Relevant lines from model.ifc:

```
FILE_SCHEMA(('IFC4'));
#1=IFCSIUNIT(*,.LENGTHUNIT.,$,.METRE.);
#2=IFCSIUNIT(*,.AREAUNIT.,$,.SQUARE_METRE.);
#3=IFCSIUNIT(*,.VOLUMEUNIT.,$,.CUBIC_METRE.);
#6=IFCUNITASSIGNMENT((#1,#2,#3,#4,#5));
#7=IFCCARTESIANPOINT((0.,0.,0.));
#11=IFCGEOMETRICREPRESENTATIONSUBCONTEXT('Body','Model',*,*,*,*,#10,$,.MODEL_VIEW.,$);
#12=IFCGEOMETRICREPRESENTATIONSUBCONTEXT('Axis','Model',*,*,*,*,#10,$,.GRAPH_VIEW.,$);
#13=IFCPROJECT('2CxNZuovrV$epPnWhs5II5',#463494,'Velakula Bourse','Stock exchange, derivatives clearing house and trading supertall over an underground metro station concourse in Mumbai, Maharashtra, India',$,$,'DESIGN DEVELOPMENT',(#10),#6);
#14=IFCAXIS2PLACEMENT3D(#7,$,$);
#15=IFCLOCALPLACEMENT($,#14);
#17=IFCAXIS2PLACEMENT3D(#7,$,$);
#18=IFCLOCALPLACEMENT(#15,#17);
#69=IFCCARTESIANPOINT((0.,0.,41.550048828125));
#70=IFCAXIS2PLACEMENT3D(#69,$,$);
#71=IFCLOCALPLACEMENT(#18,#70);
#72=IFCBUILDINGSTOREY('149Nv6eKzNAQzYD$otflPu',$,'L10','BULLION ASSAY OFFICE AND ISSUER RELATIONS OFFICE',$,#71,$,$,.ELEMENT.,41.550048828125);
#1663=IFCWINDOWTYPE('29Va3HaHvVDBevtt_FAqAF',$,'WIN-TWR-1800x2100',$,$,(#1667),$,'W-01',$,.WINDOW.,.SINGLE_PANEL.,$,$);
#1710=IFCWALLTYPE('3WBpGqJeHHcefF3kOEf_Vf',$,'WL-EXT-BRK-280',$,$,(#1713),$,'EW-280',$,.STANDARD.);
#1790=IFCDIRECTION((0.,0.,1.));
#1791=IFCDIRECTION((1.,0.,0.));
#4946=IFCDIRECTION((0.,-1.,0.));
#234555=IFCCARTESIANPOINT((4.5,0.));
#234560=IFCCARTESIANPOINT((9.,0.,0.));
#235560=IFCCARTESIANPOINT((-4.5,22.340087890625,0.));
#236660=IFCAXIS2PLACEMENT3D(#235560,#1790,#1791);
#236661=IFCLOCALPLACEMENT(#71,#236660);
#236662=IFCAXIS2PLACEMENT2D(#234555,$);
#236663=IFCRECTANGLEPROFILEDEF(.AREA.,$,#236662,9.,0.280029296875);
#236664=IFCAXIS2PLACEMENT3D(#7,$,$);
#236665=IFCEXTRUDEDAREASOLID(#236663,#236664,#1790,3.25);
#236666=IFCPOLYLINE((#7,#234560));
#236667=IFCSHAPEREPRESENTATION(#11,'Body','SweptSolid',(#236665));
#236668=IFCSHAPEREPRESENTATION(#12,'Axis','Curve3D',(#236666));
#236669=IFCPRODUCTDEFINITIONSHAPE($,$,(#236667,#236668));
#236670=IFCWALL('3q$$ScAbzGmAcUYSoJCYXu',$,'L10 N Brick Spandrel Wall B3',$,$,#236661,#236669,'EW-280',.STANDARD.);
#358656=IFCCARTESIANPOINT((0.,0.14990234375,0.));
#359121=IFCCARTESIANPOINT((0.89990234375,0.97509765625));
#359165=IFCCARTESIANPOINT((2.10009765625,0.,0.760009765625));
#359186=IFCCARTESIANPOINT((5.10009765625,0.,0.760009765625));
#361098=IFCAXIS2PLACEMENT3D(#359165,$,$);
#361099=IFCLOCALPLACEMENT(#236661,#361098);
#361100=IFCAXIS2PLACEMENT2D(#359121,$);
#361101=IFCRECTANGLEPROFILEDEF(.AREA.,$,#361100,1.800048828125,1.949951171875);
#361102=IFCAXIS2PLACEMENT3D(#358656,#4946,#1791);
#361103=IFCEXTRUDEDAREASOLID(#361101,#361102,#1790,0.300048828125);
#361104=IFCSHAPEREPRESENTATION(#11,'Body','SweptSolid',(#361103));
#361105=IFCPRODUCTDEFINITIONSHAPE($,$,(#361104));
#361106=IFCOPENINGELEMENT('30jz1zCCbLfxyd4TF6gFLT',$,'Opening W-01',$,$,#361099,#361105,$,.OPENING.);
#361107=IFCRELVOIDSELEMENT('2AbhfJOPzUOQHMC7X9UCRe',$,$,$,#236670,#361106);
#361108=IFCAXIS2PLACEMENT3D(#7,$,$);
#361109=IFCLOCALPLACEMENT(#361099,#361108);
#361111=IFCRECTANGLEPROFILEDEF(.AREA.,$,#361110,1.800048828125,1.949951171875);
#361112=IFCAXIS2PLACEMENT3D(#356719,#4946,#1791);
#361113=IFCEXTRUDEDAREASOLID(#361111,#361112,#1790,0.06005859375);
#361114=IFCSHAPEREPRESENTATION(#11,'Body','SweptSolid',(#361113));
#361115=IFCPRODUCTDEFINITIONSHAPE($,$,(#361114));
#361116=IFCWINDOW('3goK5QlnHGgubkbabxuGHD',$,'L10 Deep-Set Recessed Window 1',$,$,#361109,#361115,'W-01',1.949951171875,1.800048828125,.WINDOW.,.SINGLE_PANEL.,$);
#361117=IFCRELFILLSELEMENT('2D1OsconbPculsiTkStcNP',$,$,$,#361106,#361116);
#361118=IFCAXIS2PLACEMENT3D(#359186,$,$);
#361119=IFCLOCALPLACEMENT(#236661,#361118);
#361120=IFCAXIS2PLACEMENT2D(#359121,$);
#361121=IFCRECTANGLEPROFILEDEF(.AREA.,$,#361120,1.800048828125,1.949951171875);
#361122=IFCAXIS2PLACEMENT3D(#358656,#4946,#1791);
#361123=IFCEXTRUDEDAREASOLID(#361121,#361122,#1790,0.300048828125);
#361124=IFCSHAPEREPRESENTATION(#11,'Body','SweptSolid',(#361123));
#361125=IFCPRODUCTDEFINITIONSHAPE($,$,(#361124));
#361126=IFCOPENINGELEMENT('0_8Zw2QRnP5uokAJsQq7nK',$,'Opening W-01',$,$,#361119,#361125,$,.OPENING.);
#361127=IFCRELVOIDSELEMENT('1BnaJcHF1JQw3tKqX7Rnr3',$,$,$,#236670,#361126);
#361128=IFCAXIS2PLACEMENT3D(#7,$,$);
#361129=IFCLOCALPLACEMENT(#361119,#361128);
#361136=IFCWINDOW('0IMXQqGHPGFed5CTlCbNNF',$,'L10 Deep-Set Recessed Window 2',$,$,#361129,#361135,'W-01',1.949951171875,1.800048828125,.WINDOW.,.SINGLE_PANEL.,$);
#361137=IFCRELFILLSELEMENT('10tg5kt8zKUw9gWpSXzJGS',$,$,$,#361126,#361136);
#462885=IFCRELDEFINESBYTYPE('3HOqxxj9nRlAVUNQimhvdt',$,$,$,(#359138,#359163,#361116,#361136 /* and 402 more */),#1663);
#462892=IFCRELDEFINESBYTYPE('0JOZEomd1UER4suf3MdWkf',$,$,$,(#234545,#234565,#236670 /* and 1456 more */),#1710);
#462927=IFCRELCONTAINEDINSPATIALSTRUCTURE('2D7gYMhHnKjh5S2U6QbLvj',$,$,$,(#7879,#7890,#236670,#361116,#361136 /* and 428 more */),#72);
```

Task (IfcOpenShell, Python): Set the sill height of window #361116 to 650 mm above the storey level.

```python
import numpy as np
import ifcopenshell
import ifcopenshell.api.geometry
import ifcopenshell.geom
import ifcopenshell.util.element
import ifcopenshell.util.placement
import ifcopenshell.util.shape
import ifcopenshell.util.unit

model = ifcopenshell.open("model.ifc")
unit_scale = ifcopenshell.util.unit.calculate_unit_scale(model)

window = model.by_guid("3goK5QlnHGgubkbabxuGHD")
opening = window.FillsVoids[0].RelatingOpeningElement
storey = ifcopenshell.util.element.get_container(window, ifc_class="IfcBuildingStorey")
level = ifcopenshell.util.placement.get_local_placement(storey.ObjectPlacement)[2, 3]

# The opening's origin need not be at the sill, so measure its lowest point.
shape = ifcopenshell.geom.create_shape(ifcopenshell.geom.settings(), opening)
bottom = ifcopenshell.util.shape.get_shape_bottom_elevation(shape, shape.geometry) / unit_scale
dz = level + 0.65 / unit_scale - bottom

shift = np.array([0.0, 0.0, dz])
# The window is placed relative to its opening, so it follows when the opening moves.
matrix = ifcopenshell.util.placement.get_local_placement(opening.ObjectPlacement)
matrix[:3, 3] += shift
ifcopenshell.api.geometry.edit_object_placement(
    model, product=opening, matrix=matrix, is_si=False, should_transform_children=True
)

print(f"moved by {dz * unit_scale:+.3f} m")

model.write("model_edited.ifc")
```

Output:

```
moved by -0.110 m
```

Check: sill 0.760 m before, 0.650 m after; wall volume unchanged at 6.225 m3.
